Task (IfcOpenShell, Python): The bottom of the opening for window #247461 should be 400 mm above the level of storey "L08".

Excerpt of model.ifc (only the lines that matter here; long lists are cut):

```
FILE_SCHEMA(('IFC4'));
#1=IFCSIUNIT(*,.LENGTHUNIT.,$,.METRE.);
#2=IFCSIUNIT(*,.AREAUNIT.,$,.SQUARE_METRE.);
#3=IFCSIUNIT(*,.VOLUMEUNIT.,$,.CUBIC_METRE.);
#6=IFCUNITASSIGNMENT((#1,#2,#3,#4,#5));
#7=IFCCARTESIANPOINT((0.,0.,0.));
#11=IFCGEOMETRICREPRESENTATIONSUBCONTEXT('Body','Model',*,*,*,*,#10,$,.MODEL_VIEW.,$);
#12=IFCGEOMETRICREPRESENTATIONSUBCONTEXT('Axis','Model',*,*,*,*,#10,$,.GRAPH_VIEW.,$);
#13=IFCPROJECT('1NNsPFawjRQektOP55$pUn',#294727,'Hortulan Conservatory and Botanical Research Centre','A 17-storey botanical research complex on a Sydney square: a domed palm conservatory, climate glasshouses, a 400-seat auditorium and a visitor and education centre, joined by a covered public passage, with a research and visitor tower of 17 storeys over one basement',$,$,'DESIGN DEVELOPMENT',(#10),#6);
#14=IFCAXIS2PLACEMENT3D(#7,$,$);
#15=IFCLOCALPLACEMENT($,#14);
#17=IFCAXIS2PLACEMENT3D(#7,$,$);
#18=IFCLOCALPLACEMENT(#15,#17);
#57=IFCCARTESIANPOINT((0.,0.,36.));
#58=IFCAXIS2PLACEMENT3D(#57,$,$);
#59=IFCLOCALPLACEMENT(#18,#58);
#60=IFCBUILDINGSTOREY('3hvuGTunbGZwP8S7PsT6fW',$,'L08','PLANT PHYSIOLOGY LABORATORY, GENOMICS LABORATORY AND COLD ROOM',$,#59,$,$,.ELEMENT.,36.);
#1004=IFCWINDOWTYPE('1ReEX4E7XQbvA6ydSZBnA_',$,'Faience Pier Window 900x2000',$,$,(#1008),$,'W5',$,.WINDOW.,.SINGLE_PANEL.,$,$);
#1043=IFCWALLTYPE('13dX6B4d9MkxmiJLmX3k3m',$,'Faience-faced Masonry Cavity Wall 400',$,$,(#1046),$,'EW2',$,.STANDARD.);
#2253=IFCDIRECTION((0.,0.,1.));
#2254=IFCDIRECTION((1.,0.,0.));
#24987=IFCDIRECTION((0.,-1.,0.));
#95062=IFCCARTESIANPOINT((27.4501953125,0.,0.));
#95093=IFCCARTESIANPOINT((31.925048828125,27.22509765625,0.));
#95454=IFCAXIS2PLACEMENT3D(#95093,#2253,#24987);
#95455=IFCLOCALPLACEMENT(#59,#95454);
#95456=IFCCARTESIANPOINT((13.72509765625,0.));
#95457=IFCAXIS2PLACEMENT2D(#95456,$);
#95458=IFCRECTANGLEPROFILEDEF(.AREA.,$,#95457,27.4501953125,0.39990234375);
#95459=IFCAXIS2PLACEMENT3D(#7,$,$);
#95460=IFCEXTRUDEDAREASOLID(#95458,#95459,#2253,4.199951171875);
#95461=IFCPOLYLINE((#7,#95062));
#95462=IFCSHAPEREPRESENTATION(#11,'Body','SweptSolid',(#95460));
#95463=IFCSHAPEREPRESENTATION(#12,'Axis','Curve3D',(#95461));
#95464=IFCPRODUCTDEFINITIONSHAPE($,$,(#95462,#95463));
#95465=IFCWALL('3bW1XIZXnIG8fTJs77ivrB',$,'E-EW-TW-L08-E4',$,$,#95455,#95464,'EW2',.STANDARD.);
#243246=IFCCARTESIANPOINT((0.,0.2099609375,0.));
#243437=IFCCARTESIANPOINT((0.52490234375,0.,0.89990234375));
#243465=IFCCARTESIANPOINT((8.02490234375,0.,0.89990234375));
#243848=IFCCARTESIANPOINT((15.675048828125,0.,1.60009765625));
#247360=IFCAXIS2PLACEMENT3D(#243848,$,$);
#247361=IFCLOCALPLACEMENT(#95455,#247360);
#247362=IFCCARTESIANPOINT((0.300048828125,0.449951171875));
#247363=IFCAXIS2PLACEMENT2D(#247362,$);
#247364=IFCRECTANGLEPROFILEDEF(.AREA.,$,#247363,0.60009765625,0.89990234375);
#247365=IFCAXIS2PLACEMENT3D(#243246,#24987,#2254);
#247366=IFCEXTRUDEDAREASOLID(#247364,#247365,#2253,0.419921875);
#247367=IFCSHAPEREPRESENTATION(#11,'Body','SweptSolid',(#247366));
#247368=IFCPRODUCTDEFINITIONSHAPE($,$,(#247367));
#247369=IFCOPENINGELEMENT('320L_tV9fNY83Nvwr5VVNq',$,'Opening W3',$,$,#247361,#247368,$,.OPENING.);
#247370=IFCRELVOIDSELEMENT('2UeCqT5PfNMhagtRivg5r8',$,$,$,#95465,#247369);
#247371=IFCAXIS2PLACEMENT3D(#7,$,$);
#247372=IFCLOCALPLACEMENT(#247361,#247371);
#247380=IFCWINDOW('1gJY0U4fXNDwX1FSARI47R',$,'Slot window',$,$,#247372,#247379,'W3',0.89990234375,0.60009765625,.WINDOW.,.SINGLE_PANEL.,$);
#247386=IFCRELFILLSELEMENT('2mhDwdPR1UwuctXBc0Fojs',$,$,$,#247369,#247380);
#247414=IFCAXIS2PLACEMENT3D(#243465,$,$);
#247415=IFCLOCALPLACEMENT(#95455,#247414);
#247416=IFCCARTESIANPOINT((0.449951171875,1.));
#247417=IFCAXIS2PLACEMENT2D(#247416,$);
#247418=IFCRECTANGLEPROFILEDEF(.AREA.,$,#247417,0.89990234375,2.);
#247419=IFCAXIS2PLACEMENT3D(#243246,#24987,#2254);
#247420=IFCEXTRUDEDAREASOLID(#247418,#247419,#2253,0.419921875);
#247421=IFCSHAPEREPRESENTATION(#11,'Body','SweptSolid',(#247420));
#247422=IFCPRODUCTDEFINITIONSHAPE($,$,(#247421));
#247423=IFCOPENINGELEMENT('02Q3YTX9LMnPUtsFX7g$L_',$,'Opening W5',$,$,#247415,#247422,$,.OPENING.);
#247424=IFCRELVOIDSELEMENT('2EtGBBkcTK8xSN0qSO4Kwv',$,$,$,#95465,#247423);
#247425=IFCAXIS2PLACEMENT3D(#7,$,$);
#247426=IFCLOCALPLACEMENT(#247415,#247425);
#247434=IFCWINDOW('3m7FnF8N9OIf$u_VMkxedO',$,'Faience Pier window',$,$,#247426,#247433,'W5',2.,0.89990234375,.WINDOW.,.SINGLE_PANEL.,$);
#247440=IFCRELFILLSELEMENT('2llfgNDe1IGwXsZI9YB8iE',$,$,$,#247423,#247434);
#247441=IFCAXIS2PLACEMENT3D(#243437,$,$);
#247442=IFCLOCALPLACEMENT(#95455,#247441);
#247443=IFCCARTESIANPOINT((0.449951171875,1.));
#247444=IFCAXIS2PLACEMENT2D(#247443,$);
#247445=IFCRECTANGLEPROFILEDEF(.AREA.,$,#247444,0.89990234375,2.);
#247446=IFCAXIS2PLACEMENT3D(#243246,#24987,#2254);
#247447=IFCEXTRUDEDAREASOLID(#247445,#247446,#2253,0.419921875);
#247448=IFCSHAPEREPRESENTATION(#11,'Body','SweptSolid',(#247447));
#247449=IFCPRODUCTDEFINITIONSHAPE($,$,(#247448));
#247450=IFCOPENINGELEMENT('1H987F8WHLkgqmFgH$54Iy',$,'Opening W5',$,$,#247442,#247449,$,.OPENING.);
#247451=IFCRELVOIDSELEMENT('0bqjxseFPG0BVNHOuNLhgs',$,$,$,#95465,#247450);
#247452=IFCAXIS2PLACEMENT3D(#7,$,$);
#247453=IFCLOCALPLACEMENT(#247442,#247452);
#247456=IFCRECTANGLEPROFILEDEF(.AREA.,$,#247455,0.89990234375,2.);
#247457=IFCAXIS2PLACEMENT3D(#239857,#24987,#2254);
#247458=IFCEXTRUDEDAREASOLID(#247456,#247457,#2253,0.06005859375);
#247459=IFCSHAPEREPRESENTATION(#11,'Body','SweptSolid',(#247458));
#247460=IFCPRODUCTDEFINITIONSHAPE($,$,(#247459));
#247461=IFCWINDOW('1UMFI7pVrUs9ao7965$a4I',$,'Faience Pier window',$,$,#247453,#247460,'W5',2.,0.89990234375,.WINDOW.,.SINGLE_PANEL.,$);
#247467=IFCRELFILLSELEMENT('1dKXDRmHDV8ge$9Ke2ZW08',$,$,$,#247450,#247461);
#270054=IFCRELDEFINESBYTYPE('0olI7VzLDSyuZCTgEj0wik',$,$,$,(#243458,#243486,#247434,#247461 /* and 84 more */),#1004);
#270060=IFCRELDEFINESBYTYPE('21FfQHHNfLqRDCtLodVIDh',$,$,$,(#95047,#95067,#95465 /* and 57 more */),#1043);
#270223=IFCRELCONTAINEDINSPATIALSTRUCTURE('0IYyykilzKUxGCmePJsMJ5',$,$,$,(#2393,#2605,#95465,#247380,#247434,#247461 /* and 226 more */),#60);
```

```python
import numpy as np
import ifcopenshell
import ifcopenshell.api.geometry
import ifcopenshell.geom
import ifcopenshell.util.element
import ifcopenshell.util.placement
import ifcopenshell.util.shape
import ifcopenshell.util.unit

model = ifcopenshell.open("model.ifc")
unit_scale = ifcopenshell.util.unit.calculate_unit_scale(model)

window = model.by_guid("1UMFI7pVrUs9ao7965$a4I")
opening = window.FillsVoids[0].RelatingOpeningElement
storey = ifcopenshell.util.element.get_container(window, ifc_class="IfcBuildingStorey")
level = ifcopenshell.util.placement.get_local_placement(storey.ObjectPlacement)[2, 3]

# The opening's origin need not be at the sill, so measure its lowest point.
shape = ifcopenshell.geom.create_shape(ifcopenshell.geom.settings(), opening)
bottom = ifcopenshell.util.shape.get_shape_bottom_elevation(shape, shape.geometry) / unit_scale
dz = level + 0.4 / unit_scale - bottom

shift = np.array([0.0, 0.0, dz])
# The window is placed relative to its opening, so it follows when the opening moves.
matrix = ifcopenshell.util.placement.get_local_placement(opening.ObjectPlacement)
matrix[:3, 3] += shift
ifcopenshell.api.geometry.edit_object_placement(
    model, product=opening, matrix=matrix, is_si=False, should_transform_children=True
)

print(f"moved by {dz * unit_scale:+.3f} m")

model.write("model-out.ifc")
```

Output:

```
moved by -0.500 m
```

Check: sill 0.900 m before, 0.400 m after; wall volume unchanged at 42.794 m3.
